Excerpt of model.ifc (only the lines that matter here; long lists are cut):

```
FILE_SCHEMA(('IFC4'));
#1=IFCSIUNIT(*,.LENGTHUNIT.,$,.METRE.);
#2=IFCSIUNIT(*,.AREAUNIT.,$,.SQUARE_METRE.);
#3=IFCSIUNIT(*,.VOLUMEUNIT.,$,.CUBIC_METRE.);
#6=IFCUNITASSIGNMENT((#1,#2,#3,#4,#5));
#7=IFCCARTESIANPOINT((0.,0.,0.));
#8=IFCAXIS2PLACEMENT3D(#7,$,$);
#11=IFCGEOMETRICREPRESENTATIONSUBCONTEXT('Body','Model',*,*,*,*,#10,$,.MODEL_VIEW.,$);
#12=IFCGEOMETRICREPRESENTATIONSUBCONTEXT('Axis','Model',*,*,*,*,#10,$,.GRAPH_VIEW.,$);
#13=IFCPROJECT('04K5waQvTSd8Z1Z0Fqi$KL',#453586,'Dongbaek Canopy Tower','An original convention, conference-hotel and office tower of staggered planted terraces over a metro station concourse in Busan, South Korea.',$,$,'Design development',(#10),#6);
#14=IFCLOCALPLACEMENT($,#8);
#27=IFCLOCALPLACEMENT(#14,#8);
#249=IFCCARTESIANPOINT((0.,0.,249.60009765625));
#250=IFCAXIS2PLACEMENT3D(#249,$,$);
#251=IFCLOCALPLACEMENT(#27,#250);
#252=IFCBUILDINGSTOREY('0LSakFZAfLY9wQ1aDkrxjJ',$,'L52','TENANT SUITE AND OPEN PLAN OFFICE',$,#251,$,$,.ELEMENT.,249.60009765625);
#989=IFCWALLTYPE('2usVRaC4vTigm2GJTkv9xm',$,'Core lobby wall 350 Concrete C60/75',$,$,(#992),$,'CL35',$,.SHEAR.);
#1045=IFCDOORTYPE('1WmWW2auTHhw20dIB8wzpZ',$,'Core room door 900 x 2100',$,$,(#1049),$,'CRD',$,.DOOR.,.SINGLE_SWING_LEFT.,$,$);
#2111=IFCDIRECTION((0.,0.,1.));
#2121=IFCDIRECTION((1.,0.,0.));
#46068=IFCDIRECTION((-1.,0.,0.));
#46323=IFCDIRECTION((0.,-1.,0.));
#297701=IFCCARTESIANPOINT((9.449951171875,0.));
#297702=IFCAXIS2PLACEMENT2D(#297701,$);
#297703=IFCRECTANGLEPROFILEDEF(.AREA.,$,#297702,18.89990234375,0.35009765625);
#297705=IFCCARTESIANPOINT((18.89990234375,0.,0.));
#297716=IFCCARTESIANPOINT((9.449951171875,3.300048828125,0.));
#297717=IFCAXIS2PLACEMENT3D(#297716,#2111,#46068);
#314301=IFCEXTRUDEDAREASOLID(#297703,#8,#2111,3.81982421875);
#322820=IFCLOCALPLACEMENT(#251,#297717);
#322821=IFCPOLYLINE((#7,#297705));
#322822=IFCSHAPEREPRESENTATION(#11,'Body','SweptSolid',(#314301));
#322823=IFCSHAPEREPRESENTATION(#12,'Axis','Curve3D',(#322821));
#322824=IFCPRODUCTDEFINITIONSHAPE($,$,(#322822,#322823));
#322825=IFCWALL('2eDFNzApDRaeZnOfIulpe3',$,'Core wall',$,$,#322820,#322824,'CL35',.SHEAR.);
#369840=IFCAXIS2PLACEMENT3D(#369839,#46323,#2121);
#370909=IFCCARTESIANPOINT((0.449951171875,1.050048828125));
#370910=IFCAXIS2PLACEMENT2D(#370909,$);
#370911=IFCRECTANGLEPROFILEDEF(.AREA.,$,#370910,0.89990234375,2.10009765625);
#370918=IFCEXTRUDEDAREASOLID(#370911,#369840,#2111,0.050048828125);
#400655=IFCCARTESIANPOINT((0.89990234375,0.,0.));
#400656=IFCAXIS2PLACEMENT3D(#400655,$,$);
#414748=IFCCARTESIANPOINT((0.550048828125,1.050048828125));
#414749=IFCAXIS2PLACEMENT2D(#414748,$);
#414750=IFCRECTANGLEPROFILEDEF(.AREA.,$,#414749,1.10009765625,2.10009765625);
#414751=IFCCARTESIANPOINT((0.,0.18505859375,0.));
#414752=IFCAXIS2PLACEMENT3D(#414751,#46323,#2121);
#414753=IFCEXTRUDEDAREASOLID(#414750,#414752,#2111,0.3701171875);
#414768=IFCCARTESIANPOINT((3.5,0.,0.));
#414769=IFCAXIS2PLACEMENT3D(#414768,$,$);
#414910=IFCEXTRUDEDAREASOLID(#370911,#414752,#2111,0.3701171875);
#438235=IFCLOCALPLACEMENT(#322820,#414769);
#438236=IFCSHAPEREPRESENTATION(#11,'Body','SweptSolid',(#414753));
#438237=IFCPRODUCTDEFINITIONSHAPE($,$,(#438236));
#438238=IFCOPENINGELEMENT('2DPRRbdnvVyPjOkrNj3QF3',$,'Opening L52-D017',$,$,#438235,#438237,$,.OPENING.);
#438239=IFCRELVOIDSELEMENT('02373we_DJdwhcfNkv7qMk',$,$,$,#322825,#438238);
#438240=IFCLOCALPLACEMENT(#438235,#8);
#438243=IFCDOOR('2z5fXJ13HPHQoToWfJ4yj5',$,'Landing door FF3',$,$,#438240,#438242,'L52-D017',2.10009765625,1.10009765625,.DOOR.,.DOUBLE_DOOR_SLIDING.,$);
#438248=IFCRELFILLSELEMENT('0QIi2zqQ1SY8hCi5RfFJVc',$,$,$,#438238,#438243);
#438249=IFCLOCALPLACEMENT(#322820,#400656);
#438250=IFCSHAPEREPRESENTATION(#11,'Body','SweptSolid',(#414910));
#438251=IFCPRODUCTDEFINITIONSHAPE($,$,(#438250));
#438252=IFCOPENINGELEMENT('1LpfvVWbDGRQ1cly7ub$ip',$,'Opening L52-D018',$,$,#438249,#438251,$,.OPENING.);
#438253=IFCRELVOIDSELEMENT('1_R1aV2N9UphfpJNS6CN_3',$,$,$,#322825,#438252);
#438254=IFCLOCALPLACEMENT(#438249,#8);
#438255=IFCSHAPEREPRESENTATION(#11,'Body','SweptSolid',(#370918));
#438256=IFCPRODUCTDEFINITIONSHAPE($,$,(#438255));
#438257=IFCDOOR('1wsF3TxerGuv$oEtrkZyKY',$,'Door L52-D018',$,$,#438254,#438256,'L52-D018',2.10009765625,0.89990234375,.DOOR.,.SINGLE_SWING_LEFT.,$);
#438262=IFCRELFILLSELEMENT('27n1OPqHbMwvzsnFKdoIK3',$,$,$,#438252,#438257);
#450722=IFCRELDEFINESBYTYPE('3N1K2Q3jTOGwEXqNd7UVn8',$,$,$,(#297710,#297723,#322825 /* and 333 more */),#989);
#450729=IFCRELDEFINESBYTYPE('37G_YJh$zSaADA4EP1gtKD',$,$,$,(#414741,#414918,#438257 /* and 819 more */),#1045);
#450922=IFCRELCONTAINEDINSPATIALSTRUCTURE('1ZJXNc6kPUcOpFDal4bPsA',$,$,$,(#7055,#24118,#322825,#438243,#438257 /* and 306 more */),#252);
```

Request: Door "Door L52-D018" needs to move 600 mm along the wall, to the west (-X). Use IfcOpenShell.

```python
import ifcopenshell
import ifcopenshell.api.geometry
import ifcopenshell.util.placement
import ifcopenshell.util.unit

model = ifcopenshell.open("model.ifc")
unit_scale = ifcopenshell.util.unit.calculate_unit_scale(model)

door = model.by_guid("1wsF3TxerGuv$oEtrkZyKY")
opening = door.FillsVoids[0].RelatingOpeningElement
wall = opening.VoidsElements[0].RelatingBuildingElement

wall_matrix = ifcopenshell.util.placement.get_local_placement(wall.ObjectPlacement)
shift = wall_matrix[:3, 0] * 0.6 / unit_scale
before = ifcopenshell.util.placement.get_local_placement(door.ObjectPlacement)[:3, 3].copy()

# The door is placed relative to its opening, so it follows when the opening moves.
matrix = ifcopenshell.util.placement.get_local_placement(opening.ObjectPlacement)
matrix[:3, 3] += shift
ifcopenshell.api.geometry.edit_object_placement(
    model, product=opening, matrix=matrix, is_si=False, should_transform_children=True
)

after = ifcopenshell.util.placement.get_local_placement(door.ObjectPlacement)[:3, 3]
print("door moved by", (after - before).round(3) + 0.0)

model.write("model_v2.ifc")
```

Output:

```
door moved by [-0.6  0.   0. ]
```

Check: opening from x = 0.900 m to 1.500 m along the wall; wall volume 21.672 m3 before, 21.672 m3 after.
